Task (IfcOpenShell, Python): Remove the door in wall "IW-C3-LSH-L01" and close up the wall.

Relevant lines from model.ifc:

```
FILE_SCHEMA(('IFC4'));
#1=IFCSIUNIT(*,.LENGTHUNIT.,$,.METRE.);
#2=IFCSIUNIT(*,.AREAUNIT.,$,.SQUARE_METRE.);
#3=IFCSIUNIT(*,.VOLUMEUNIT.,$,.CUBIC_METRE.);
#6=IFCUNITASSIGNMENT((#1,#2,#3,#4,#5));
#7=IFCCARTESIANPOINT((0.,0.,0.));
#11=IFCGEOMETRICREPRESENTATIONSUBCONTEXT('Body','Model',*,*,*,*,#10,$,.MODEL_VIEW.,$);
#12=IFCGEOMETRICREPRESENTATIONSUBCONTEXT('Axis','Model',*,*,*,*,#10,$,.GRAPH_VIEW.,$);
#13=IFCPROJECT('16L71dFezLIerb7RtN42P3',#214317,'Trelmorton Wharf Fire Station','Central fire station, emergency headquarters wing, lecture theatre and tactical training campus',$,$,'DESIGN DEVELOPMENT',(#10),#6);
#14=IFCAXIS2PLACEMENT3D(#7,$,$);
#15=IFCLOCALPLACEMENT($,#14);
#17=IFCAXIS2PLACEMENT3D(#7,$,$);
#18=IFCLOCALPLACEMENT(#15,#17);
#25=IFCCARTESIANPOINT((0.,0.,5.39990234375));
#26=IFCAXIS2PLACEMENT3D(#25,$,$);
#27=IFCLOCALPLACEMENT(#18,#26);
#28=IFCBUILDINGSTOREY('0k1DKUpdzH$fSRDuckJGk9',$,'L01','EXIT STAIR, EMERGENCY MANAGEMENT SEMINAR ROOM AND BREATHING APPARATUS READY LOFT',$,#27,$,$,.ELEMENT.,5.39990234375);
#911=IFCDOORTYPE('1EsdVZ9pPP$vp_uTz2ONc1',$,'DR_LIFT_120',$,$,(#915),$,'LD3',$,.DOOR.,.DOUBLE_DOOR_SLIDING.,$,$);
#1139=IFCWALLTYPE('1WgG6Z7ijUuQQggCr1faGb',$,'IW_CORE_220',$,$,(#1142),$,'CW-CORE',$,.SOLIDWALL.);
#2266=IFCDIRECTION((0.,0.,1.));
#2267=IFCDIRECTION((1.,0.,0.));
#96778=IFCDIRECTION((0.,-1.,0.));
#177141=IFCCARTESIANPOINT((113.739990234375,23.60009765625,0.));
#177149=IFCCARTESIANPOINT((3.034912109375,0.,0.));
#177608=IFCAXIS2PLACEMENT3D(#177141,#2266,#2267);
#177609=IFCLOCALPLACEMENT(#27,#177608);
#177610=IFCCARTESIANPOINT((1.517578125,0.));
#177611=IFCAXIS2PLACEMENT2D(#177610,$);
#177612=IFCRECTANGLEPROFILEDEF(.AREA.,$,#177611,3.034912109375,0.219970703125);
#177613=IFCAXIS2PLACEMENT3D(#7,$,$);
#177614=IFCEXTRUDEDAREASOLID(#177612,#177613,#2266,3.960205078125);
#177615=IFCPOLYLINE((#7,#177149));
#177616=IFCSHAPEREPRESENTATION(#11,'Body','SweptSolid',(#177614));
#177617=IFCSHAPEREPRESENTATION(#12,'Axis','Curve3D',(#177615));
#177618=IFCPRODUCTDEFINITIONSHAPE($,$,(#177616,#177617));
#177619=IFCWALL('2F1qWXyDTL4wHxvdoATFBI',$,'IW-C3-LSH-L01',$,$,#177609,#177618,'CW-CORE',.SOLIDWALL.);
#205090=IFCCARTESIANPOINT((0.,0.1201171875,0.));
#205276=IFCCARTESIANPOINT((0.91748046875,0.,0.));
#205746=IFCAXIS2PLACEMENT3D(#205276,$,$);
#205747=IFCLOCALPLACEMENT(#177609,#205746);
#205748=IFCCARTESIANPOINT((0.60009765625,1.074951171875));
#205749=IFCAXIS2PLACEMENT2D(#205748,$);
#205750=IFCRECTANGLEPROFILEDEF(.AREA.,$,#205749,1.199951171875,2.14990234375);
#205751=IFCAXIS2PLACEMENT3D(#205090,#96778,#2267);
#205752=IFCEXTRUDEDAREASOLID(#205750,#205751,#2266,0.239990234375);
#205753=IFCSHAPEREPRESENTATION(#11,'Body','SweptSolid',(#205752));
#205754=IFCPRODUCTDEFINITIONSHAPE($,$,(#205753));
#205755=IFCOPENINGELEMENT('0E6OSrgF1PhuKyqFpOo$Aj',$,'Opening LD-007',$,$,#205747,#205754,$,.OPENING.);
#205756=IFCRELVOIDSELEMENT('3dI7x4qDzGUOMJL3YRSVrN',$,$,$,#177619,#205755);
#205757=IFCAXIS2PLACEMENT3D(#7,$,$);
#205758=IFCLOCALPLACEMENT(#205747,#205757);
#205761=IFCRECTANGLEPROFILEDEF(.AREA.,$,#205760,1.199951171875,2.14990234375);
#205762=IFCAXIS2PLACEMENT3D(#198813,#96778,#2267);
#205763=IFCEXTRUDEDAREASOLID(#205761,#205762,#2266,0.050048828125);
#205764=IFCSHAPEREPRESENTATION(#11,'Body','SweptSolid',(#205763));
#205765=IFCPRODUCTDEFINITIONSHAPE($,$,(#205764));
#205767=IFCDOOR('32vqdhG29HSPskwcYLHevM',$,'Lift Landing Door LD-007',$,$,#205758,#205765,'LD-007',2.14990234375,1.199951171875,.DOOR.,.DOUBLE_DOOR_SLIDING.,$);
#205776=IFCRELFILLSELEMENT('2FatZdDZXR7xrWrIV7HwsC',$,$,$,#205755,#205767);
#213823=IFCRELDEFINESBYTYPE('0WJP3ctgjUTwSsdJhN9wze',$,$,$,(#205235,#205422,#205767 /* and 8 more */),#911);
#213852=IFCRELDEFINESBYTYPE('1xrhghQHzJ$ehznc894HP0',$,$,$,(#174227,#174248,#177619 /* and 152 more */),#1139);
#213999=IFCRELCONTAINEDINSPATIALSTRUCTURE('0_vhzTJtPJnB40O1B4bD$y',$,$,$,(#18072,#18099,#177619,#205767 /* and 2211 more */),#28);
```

```python
import ifcopenshell
import ifcopenshell.api.feature
import ifcopenshell.api.root
import ifcopenshell.geom
import ifcopenshell.util.shape

model = ifcopenshell.open("model.ifc")
settings = ifcopenshell.geom.settings()


def volume(element):
    """Net volume in cubic metres, openings subtracted."""
    shape = ifcopenshell.geom.create_shape(settings, element)
    return ifcopenshell.util.shape.get_volume(shape.geometry)


door = model.by_guid("32vqdhG29HSPskwcYLHevM")
opening = door.FillsVoids[0].RelatingOpeningElement
wall = opening.VoidsElements[0].RelatingBuildingElement
before = volume(wall)

ifcopenshell.api.root.remove_product(model, product=door)
ifcopenshell.api.feature.remove_feature(model, feature=opening)

after = volume(wall)

print(f"wall volume {before:.3f} -> {after:.3f} m3")

model.write("model_edited.ifc")
```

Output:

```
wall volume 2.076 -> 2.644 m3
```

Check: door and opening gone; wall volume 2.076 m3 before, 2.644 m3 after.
